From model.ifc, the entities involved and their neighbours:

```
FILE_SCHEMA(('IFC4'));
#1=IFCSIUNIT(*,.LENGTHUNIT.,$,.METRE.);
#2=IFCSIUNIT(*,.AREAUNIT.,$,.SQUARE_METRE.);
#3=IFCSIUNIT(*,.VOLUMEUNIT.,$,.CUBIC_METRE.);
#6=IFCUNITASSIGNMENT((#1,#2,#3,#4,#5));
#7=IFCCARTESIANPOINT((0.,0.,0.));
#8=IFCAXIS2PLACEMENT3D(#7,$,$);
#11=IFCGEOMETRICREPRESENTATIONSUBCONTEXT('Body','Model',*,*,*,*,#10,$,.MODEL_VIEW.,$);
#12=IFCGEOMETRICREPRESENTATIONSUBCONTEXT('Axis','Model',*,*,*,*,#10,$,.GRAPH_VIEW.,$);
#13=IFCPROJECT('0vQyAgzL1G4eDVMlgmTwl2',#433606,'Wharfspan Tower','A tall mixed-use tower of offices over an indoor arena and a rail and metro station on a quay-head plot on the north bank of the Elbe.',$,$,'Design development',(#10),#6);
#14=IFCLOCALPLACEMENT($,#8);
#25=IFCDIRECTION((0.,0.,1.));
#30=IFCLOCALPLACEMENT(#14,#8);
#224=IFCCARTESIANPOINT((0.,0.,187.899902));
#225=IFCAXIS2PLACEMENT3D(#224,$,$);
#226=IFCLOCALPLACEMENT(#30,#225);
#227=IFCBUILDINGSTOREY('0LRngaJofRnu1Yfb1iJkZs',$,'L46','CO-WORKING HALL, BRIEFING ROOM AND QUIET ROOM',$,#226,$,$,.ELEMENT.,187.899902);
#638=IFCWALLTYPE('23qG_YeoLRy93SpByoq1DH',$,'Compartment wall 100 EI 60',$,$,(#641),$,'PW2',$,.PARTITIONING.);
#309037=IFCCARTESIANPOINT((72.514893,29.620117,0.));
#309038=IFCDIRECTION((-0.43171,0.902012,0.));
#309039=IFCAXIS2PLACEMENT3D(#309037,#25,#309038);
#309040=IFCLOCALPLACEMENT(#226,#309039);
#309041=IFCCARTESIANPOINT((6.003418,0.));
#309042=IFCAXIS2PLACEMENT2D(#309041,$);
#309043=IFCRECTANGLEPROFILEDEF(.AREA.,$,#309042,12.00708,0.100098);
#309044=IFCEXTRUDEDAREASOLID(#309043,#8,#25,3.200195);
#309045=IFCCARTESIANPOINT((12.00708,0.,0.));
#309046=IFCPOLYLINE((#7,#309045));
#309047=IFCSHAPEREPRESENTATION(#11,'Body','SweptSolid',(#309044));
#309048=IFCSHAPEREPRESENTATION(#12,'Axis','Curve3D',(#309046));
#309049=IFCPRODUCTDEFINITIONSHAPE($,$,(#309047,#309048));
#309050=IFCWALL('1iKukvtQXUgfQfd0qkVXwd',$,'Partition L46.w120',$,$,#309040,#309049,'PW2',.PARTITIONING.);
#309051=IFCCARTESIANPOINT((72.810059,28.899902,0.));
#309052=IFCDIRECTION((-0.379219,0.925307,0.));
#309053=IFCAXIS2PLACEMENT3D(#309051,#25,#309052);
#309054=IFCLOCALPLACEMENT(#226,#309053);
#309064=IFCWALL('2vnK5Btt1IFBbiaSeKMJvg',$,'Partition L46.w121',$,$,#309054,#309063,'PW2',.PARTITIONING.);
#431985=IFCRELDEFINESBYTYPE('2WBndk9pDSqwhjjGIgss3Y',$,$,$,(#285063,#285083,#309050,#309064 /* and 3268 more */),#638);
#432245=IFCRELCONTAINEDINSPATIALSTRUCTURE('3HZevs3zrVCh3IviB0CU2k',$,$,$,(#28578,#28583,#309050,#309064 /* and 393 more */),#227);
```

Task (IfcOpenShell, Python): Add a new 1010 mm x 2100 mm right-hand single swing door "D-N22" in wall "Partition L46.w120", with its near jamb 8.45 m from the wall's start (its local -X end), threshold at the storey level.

```python
import numpy as np
import ifcopenshell
import ifcopenshell.api.feature
import ifcopenshell.api.geometry
import ifcopenshell.api.root
import ifcopenshell.api.spatial
import ifcopenshell.geom
import ifcopenshell.util.element
import ifcopenshell.util.placement
import ifcopenshell.util.representation
import ifcopenshell.util.shape
import ifcopenshell.util.unit

model = ifcopenshell.open("model.ifc")
unit_scale = ifcopenshell.util.unit.calculate_unit_scale(model)
settings = ifcopenshell.geom.settings()


def volume(element):
    """Net volume in cubic metres, openings subtracted."""
    shape = ifcopenshell.geom.create_shape(settings, element)
    return ifcopenshell.util.shape.get_volume(shape.geometry)


wall = model.by_guid("1iKukvtQXUgfQfd0qkVXwd")
storey = ifcopenshell.util.element.get_container(wall, ifc_class="IfcBuildingStorey")
context = ifcopenshell.util.representation.get_context(model, "Model", "Body", "MODEL_VIEW")
before = volume(wall)

width, height, from_end, sill = 1.01, 2.1, 8.45, 0.0  # metres

# The wall runs along its own X axis, and the end named is its -X end.
wall_shape = ifcopenshell.geom.create_shape(settings, wall)
x, y, z = ifcopenshell.util.shape.get_vertices(wall_shape.geometry).T
start = x.min() + from_end
face, thickness = float(y.min()), float(y.max() - y.min())
wall_matrix = ifcopenshell.util.placement.get_local_placement(wall.ObjectPlacement)
level = ifcopenshell.util.placement.get_local_placement(storey.ObjectPlacement)[2, 3]


def in_wall(x, y):
    """Placement at x, y metres in the wall's axes, at sill height."""
    matrix = wall_matrix.copy()
    matrix[:, 3] = wall_matrix @ np.array([x / unit_scale, y / unit_scale, 0.0, 1.0])
    matrix[2, 3] = level + sill / unit_scale
    return matrix


# Opening: a box that overshoots both wall faces by 50 mm.
opening = ifcopenshell.api.root.create_entity(model, ifc_class="IfcOpeningElement", predefined_type="OPENING")
box = ifcopenshell.api.geometry.add_wall_representation(
    model, context=context, length=width, height=height, thickness=thickness + 0.1
)
ifcopenshell.api.geometry.assign_representation(model, product=opening, representation=box)
ifcopenshell.api.geometry.edit_object_placement(model, product=opening, matrix=in_wall(start, face - 0.05), is_si=False)
ifcopenshell.api.feature.add_feature(model, feature=opening, element=wall)

door = ifcopenshell.api.root.create_entity(model, ifc_class="IfcDoor", name="D-N22", predefined_type="DOOR")
door.OverallWidth, door.OverallHeight = width / unit_scale, height / unit_scale
door.OperationType = "SINGLE_SWING_RIGHT"
body = ifcopenshell.api.geometry.add_door_representation(
    model,
    context=context,
    overall_width=door.OverallWidth,
    overall_height=door.OverallHeight,
    operation_type="SINGLE_SWING_RIGHT",
    lining_properties={"LiningDepth": thickness / unit_scale, "ThresholdDepth": thickness / unit_scale},
)
ifcopenshell.api.geometry.assign_representation(model, product=door, representation=body)
ifcopenshell.api.spatial.assign_container(model, products=[door], relating_structure=storey)
ifcopenshell.api.feature.add_filling(model, opening=opening, element=door)

# The lining spans the wall, so the door starts at the wall face.
ifcopenshell.api.geometry.edit_object_placement(model, product=door, matrix=in_wall(start, face), is_si=False)

after = volume(wall)

print(f"wall volume {before:.3f} -> {after:.3f} m3")

model.write("model_rev.ifc")
```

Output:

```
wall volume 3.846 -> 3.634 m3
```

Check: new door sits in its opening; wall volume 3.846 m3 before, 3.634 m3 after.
